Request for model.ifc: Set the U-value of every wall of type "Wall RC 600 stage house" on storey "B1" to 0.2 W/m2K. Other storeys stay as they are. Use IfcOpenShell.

First a look at what the model holds.

```python
import ifcopenshell
import ifcopenshell.util.element

model = ifcopenshell.open("model.ifc")
print(model.schema)
storey = next(s for s in model.by_type("IfcBuildingStorey") if s.Name == "B1")
walls = [e for e in ifcopenshell.util.element.get_decomposition(storey) if e.is_a("IfcWall")]
seen = {}
for e in walls:
    element_type = ifcopenshell.util.element.get_type(e)
    key = (element_type.Name if element_type != e and element_type else None, ifcopenshell.util.element.get_pset(e, "Pset_WallCommon", "ThermalTransmittance"))
    seen[key] = seen.get(key, 0) + 1
for (name, value), count in sorted(seen.items(), key=str):
    print(count, "x", name, "|", value)
```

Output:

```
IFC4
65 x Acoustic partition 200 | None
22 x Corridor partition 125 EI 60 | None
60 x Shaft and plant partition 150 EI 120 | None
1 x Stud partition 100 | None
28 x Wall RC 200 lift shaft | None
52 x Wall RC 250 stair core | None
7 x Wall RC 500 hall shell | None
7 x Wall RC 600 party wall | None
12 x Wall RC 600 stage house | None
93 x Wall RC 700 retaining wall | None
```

```python
import ifcopenshell
import ifcopenshell.api.pset
import ifcopenshell.util.element

model = ifcopenshell.open("model.ifc")

storey = next(s for s in model.by_type("IfcBuildingStorey") if s.Name == "B1")
walls = [e for e in ifcopenshell.util.element.get_decomposition(storey) if e.is_a("IfcWall")]

count = 0
for e in walls:
    element_type = ifcopenshell.util.element.get_type(e)
    if element_type in (None, e) or element_type.Name != "Wall RC 600 stage house":
        continue
    # add_pset returns the element's existing set when there is one.
    pset = ifcopenshell.api.pset.add_pset(model, product=e, name="Pset_WallCommon")
    ifcopenshell.api.pset.edit_pset(model, pset=pset, properties={"ThermalTransmittance": 0.2})
    count += 1

print(count, "walls updated")

model.write("model_updated.ifc")
```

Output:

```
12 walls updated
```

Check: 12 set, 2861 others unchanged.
